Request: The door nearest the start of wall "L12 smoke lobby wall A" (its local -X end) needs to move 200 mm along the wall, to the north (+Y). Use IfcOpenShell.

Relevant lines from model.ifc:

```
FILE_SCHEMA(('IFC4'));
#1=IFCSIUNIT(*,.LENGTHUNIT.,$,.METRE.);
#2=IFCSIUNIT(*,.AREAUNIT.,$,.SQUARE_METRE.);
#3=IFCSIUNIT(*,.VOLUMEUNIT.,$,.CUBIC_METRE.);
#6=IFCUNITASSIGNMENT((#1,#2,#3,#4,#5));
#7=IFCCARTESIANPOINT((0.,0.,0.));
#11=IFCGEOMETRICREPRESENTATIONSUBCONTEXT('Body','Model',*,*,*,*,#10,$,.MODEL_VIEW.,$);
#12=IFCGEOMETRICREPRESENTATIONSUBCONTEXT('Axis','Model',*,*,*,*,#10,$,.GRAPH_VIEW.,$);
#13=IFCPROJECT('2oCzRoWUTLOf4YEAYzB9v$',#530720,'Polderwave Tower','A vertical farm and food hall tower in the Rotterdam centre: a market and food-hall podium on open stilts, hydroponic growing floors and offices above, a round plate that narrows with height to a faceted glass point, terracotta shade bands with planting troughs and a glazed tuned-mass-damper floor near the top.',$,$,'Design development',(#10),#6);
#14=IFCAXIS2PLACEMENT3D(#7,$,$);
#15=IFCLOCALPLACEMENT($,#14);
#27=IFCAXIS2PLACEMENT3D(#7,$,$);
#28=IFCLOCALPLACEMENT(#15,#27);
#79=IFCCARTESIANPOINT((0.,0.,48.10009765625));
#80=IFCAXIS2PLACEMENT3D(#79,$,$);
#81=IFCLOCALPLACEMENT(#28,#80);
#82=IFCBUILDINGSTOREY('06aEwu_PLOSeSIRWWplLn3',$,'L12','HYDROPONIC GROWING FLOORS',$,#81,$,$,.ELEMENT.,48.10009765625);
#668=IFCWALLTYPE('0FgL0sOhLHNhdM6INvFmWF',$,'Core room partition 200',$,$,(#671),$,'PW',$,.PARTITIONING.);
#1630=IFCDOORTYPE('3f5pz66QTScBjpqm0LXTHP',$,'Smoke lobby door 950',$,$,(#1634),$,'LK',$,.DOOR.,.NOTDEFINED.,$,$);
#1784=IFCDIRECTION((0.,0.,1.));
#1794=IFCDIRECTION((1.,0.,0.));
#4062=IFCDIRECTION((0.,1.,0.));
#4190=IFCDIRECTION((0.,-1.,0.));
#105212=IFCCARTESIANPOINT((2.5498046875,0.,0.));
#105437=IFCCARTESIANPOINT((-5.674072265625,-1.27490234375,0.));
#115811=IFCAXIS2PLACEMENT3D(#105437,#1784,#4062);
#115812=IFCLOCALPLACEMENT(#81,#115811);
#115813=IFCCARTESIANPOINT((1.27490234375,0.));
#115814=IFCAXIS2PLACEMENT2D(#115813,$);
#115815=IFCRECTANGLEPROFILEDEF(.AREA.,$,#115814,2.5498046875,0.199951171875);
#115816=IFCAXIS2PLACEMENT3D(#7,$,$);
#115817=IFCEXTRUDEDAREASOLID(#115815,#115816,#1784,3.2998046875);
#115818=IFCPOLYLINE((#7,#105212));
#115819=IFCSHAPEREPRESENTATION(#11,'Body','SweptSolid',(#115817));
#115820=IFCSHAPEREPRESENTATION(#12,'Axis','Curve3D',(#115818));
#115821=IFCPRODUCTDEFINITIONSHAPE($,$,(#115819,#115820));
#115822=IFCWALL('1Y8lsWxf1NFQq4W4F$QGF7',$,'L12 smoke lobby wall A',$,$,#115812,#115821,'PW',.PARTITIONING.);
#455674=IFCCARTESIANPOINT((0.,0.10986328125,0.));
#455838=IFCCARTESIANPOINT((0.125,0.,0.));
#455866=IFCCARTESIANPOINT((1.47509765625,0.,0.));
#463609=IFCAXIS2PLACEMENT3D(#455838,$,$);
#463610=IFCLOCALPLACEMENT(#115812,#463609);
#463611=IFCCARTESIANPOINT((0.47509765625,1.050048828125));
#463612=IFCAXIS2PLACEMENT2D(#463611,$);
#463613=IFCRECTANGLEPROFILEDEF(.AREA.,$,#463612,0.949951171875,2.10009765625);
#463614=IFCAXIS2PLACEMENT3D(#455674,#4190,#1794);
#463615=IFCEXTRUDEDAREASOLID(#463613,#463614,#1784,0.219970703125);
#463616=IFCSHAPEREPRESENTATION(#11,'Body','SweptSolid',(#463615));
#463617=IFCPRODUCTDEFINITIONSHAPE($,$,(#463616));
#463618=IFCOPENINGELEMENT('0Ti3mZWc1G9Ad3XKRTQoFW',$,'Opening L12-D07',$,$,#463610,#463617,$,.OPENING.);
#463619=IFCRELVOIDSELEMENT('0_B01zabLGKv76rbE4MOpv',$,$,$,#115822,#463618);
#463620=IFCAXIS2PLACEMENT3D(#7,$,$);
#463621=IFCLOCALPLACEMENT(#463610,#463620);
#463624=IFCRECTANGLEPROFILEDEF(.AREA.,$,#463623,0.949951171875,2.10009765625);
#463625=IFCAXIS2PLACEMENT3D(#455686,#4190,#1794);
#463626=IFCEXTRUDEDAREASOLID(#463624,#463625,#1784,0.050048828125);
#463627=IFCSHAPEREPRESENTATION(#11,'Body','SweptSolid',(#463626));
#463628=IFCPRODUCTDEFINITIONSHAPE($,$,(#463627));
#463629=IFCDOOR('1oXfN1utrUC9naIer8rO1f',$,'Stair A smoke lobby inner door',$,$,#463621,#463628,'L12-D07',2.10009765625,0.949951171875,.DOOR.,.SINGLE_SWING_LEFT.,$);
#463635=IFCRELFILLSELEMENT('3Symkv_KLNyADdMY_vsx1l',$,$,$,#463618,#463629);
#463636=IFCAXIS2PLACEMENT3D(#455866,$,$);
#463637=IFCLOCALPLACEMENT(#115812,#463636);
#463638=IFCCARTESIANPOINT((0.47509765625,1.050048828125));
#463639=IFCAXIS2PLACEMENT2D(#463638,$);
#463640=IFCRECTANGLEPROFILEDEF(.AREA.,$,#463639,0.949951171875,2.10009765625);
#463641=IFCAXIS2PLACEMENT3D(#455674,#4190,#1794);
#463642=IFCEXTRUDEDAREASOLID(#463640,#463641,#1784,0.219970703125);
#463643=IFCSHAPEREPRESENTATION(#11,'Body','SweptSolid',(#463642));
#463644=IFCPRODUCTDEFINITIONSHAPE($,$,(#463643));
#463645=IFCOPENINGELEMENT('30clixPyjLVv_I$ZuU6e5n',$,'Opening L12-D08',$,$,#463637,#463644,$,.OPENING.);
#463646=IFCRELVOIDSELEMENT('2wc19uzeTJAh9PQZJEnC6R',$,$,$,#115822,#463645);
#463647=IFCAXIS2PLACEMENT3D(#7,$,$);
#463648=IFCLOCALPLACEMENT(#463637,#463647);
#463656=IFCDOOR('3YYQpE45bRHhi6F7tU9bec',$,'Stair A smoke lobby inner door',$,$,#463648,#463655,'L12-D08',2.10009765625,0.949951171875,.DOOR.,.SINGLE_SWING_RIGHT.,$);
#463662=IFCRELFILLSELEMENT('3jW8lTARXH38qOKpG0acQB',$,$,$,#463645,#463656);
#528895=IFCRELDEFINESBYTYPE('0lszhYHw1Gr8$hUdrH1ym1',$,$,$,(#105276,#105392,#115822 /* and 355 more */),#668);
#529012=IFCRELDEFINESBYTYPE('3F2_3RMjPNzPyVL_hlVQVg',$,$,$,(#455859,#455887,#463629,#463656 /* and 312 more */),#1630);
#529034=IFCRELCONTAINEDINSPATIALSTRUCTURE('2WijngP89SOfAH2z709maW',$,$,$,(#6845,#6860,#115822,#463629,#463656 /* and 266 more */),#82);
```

```python
import ifcopenshell
import ifcopenshell.api.geometry
import ifcopenshell.util.placement

model = ifcopenshell.open("model.ifc")

door = model.by_guid("1oXfN1utrUC9naIer8rO1f")
opening = door.FillsVoids[0].RelatingOpeningElement
wall = opening.VoidsElements[0].RelatingBuildingElement

wall_matrix = ifcopenshell.util.placement.get_local_placement(wall.ObjectPlacement)
shift = wall_matrix[:3, 0] * 0.2
before = ifcopenshell.util.placement.get_local_placement(door.ObjectPlacement)[:3, 3].copy()

# The door is placed relative to its opening, so it follows when the opening moves.
matrix = ifcopenshell.util.placement.get_local_placement(opening.ObjectPlacement)
matrix[:3, 3] += shift
ifcopenshell.api.geometry.edit_object_placement(
    model, product=opening, matrix=matrix, is_si=False, should_transform_children=True
)

after = ifcopenshell.util.placement.get_local_placement(door.ObjectPlacement)[:3, 3]
print("door moved by", (after - before).round(3) + 0.0)

model.write("model_rev.ifc")
```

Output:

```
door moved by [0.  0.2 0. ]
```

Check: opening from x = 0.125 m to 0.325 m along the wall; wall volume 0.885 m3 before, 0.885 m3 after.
